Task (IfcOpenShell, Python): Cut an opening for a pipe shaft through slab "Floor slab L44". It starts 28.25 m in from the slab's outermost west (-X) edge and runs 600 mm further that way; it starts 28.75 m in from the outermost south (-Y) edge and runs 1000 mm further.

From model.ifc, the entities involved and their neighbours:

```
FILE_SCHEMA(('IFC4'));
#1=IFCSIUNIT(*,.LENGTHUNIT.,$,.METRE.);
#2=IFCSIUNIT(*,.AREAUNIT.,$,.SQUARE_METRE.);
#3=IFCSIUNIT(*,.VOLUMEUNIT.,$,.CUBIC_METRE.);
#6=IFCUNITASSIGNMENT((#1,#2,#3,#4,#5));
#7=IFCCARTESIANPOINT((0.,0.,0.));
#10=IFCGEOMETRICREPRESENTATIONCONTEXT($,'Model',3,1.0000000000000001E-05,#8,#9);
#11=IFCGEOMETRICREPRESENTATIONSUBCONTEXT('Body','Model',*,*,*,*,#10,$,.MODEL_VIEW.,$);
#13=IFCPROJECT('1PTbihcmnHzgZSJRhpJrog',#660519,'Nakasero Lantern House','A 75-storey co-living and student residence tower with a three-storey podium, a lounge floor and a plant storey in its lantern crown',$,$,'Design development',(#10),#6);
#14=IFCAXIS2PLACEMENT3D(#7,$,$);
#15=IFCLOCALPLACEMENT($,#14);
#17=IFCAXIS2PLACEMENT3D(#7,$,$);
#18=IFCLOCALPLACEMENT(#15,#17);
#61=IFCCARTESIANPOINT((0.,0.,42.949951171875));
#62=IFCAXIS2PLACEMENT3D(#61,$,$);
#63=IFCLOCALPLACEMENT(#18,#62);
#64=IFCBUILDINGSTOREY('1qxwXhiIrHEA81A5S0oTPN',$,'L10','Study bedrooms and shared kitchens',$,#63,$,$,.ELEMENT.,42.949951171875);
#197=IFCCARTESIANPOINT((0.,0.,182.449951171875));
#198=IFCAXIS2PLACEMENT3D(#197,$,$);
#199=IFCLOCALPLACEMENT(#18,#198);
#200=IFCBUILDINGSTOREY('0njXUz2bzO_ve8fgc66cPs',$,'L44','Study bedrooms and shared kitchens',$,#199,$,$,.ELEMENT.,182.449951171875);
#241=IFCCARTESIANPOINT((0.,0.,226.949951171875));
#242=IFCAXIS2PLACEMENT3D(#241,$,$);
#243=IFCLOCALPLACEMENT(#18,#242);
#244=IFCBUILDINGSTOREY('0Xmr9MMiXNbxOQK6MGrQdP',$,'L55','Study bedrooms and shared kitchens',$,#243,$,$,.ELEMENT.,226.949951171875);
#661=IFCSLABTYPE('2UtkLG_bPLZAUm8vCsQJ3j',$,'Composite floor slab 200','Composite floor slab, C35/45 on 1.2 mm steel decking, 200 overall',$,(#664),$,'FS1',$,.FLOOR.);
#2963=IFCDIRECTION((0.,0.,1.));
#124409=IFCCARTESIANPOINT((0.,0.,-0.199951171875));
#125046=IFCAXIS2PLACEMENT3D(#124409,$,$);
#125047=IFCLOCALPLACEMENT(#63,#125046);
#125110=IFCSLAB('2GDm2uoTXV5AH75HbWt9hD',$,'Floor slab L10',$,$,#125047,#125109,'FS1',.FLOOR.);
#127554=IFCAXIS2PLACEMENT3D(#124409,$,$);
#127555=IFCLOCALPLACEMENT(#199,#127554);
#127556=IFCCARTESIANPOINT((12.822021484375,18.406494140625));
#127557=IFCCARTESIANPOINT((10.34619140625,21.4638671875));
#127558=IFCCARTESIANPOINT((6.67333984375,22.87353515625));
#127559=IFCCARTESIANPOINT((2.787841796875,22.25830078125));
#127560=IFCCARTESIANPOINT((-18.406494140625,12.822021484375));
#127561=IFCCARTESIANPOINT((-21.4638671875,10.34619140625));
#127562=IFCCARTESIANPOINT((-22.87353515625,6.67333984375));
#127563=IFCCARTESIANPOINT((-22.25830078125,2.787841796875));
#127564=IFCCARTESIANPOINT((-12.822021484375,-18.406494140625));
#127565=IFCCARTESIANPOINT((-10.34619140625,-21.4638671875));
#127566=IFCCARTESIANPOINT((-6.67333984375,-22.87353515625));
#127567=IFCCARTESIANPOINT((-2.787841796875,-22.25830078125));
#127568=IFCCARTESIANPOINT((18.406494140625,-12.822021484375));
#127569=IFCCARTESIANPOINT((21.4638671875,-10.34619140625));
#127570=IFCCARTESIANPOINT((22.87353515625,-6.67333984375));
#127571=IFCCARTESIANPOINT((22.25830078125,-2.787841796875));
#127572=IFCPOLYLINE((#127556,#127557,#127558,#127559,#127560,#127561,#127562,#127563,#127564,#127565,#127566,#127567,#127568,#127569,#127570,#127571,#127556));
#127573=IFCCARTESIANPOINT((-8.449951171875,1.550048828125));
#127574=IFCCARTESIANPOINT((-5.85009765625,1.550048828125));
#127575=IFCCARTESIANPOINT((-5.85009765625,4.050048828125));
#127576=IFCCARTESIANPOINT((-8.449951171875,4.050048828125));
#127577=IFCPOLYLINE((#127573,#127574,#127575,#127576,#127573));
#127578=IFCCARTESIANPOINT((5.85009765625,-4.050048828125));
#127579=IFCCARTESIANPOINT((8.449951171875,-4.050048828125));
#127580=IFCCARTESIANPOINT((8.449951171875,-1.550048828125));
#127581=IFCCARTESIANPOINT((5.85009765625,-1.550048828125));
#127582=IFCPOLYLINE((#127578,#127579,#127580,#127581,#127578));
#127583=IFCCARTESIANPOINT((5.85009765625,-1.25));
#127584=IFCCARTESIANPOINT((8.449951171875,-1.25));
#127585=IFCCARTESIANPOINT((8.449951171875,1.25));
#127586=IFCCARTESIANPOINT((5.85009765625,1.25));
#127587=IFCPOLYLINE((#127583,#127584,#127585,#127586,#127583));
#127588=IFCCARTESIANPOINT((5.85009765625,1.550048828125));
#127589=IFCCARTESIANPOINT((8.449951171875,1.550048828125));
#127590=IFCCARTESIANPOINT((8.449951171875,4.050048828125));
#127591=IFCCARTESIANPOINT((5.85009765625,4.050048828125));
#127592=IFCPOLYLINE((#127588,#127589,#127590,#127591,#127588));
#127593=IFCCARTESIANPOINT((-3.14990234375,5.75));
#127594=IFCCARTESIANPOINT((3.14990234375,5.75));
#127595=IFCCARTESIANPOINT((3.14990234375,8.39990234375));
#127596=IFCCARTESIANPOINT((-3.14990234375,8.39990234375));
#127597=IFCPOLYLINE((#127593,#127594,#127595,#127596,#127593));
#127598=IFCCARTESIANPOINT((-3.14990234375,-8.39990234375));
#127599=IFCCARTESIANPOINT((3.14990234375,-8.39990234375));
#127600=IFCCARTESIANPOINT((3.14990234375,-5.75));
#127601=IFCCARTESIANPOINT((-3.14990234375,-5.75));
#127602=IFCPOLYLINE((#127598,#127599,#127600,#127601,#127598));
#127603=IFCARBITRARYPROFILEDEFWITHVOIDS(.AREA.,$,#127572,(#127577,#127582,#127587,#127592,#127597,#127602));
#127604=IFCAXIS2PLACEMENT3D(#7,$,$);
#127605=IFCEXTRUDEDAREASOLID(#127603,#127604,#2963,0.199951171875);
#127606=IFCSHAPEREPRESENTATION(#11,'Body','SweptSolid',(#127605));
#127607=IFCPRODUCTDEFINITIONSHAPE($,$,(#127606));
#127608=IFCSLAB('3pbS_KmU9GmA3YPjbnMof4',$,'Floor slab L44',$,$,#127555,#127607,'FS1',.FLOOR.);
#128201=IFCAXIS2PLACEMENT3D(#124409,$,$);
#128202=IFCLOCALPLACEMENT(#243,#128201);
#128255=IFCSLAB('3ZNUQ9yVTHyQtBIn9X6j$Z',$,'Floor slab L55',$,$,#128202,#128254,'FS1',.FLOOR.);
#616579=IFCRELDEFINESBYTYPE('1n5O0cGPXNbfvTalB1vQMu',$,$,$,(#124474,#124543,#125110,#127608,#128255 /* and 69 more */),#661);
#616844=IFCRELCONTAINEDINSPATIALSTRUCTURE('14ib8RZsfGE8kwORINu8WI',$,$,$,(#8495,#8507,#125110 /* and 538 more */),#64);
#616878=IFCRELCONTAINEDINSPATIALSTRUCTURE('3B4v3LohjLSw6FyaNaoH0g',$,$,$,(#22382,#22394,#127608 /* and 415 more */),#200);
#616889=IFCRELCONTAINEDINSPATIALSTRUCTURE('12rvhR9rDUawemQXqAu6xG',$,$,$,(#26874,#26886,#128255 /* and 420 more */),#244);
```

```python
import numpy as np
import ifcopenshell
import ifcopenshell.api.feature
import ifcopenshell.api.geometry
import ifcopenshell.api.root
import ifcopenshell.geom
import ifcopenshell.util.placement
import ifcopenshell.util.representation
import ifcopenshell.util.shape
import ifcopenshell.util.unit

model = ifcopenshell.open("model.ifc")
unit_scale = ifcopenshell.util.unit.calculate_unit_scale(model)
settings = ifcopenshell.geom.settings()


def volume(element):
    """Net volume in cubic metres, openings subtracted."""
    shape = ifcopenshell.geom.create_shape(settings, element)
    return ifcopenshell.util.shape.get_volume(shape.geometry)


slab = model.by_guid("3pbS_KmU9GmA3YPjbnMof4")
before = volume(slab)

# Extent in the slab's own axes, in metres. The edges named are its -X and -Y sides.
slab_shape = ifcopenshell.geom.create_shape(settings, slab)
vertices = ifcopenshell.util.shape.get_vertices(slab_shape.geometry)
x_min, y_min, bottom = vertices.min(axis=0)
top = vertices[:, 2].max()

opening = ifcopenshell.api.root.create_entity(model, ifc_class="IfcOpeningElement", name="Pipe shaft opening", predefined_type="OPENING")
context = ifcopenshell.util.representation.get_context(model, "Model", "Body", "MODEL_VIEW")
width, depth = 0.6, 1
outline = [(0.0, 0.0), (width, 0.0), (width, depth), (0.0, depth), (0.0, 0.0)]
# Overshoot both faces by 50 mm so the cut is clean.
shape = ifcopenshell.api.geometry.add_slab_representation(
    model, context=context, depth=top - bottom + 0.1, polyline=outline
)
ifcopenshell.api.geometry.assign_representation(model, product=opening, representation=shape)

matrix = ifcopenshell.util.placement.get_local_placement(slab.ObjectPlacement)
matrix[:, 3] = matrix @ np.append(np.array([x_min + 28.25, y_min + 28.75, bottom - 0.05]) / unit_scale, 1.0)
ifcopenshell.api.geometry.edit_object_placement(model, product=opening, matrix=matrix, is_si=False)
ifcopenshell.api.feature.add_feature(model, feature=opening, element=slab)

after = volume(slab)

print(f"slab volume {before:.3f} -> {after:.3f} m3")

model.write("model_updated.ifc")
```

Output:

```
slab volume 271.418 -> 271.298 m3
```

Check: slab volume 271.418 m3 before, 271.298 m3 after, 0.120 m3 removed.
